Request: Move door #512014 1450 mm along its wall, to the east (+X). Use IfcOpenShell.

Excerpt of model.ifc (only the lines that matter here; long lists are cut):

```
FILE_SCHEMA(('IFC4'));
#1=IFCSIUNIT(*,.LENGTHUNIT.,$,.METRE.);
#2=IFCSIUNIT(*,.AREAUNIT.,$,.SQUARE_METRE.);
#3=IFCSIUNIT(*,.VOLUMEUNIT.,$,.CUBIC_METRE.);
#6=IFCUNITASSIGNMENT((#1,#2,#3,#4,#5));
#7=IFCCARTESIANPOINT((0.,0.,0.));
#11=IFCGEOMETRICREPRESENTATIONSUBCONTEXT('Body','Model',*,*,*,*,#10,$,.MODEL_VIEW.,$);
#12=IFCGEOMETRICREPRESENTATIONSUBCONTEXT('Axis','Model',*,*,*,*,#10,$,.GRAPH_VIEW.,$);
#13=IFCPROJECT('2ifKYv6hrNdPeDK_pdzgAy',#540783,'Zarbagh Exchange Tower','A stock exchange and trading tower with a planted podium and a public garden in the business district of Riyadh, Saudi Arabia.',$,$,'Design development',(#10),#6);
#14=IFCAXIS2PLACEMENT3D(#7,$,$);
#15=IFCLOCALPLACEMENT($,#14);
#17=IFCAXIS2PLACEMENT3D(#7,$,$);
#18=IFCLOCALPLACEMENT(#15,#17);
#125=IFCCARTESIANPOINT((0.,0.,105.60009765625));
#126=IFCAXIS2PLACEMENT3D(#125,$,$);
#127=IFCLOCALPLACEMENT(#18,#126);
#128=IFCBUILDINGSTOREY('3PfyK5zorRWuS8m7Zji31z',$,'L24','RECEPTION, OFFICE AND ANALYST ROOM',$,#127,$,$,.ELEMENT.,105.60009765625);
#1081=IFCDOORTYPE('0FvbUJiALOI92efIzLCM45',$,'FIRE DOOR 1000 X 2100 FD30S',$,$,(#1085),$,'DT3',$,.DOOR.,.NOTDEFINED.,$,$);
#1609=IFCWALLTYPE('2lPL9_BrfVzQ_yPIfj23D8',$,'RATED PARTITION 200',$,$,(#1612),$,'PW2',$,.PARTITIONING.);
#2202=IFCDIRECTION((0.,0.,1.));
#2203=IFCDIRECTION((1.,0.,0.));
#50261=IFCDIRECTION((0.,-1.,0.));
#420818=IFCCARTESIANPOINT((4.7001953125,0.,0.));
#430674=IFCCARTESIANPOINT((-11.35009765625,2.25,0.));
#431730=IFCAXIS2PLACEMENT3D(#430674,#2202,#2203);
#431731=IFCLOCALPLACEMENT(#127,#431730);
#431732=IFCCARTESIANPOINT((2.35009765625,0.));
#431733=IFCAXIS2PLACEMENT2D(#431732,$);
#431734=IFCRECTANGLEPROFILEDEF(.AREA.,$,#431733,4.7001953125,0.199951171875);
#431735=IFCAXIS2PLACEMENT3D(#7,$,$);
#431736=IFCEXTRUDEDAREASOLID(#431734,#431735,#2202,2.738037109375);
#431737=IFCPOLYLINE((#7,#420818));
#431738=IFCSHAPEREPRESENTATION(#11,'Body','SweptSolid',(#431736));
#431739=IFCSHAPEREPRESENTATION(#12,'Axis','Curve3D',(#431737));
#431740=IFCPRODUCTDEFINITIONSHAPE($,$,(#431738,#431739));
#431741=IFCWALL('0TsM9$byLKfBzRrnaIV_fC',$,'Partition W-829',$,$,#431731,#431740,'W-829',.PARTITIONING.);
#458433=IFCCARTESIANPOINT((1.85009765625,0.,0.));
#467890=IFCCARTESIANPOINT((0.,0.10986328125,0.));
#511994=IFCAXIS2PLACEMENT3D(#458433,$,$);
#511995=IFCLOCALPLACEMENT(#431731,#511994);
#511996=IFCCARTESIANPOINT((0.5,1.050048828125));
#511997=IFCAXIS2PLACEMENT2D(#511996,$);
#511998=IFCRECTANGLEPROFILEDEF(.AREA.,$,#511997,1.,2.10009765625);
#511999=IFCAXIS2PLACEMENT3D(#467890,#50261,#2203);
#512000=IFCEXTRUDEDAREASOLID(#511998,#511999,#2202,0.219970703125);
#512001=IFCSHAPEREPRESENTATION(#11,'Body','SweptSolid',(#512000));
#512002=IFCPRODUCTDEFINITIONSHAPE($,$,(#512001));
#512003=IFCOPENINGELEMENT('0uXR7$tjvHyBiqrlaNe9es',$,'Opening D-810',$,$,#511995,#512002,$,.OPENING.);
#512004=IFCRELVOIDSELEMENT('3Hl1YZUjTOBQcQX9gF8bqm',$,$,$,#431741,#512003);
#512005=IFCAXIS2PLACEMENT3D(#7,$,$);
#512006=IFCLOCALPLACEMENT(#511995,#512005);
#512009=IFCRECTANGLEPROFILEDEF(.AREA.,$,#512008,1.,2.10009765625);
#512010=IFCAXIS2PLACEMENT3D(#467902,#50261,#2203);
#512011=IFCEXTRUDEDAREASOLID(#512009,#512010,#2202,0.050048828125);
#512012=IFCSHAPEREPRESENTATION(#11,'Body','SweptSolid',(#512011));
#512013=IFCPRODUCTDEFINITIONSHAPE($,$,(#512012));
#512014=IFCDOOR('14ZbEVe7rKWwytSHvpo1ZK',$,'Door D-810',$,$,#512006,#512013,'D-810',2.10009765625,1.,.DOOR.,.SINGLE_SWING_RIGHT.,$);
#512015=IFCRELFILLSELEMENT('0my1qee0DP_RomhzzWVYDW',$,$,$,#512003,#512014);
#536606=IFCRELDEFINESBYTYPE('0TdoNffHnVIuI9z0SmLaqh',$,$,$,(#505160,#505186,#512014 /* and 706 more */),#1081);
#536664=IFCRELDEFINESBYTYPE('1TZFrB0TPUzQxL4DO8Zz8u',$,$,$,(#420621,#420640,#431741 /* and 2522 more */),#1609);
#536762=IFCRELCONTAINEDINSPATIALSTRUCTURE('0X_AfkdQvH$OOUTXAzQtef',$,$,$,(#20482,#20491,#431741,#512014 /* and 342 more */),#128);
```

```python
import ifcopenshell
import ifcopenshell.api.geometry
import ifcopenshell.util.placement
import ifcopenshell.util.unit

model = ifcopenshell.open("model.ifc")
unit_scale = ifcopenshell.util.unit.calculate_unit_scale(model)

door = model.by_guid("14ZbEVe7rKWwytSHvpo1ZK")
opening = door.FillsVoids[0].RelatingOpeningElement
wall = opening.VoidsElements[0].RelatingBuildingElement

wall_matrix = ifcopenshell.util.placement.get_local_placement(wall.ObjectPlacement)
shift = wall_matrix[:3, 0] * 1.45 / unit_scale
before = ifcopenshell.util.placement.get_local_placement(door.ObjectPlacement)[:3, 3].copy()

# The door is placed relative to its opening, so it follows when the opening moves.
matrix = ifcopenshell.util.placement.get_local_placement(opening.ObjectPlacement)
matrix[:3, 3] += shift
ifcopenshell.api.geometry.edit_object_placement(
    model, product=opening, matrix=matrix, is_si=False, should_transform_children=True
)

after = ifcopenshell.util.placement.get_local_placement(door.ObjectPlacement)[:3, 3]
print("door moved by", (after - before).round(3) + 0.0)

model.write("model_rev.ifc")
```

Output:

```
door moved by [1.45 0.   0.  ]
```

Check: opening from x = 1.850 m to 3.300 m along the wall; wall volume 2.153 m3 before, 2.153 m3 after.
